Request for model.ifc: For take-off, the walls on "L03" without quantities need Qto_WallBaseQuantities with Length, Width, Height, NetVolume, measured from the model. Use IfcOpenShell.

First a look at what the model holds.

```python
import ifcopenshell
import ifcopenshell.util.element
import ifcopenshell.util.unit

model = ifcopenshell.open("model.ifc")
print(model.schema)
for unit_type in ("LENGTHUNIT", "AREAUNIT", "VOLUMEUNIT"):
    print(unit_type, ifcopenshell.util.unit.calculate_unit_scale(model, unit_type))
storey = next(s for s in model.by_type("IfcBuildingStorey") if s.Name == "L03")
walls = [e for e in ifcopenshell.util.element.get_decomposition(storey) if e.is_a("IfcWall")]
for e in sorted(walls, key=lambda e: e.id()):
    print(e.id(), e.is_a(), e.Name, list(ifcopenshell.util.element.get_psets(e, qtos_only=True)), sep=" | ")
```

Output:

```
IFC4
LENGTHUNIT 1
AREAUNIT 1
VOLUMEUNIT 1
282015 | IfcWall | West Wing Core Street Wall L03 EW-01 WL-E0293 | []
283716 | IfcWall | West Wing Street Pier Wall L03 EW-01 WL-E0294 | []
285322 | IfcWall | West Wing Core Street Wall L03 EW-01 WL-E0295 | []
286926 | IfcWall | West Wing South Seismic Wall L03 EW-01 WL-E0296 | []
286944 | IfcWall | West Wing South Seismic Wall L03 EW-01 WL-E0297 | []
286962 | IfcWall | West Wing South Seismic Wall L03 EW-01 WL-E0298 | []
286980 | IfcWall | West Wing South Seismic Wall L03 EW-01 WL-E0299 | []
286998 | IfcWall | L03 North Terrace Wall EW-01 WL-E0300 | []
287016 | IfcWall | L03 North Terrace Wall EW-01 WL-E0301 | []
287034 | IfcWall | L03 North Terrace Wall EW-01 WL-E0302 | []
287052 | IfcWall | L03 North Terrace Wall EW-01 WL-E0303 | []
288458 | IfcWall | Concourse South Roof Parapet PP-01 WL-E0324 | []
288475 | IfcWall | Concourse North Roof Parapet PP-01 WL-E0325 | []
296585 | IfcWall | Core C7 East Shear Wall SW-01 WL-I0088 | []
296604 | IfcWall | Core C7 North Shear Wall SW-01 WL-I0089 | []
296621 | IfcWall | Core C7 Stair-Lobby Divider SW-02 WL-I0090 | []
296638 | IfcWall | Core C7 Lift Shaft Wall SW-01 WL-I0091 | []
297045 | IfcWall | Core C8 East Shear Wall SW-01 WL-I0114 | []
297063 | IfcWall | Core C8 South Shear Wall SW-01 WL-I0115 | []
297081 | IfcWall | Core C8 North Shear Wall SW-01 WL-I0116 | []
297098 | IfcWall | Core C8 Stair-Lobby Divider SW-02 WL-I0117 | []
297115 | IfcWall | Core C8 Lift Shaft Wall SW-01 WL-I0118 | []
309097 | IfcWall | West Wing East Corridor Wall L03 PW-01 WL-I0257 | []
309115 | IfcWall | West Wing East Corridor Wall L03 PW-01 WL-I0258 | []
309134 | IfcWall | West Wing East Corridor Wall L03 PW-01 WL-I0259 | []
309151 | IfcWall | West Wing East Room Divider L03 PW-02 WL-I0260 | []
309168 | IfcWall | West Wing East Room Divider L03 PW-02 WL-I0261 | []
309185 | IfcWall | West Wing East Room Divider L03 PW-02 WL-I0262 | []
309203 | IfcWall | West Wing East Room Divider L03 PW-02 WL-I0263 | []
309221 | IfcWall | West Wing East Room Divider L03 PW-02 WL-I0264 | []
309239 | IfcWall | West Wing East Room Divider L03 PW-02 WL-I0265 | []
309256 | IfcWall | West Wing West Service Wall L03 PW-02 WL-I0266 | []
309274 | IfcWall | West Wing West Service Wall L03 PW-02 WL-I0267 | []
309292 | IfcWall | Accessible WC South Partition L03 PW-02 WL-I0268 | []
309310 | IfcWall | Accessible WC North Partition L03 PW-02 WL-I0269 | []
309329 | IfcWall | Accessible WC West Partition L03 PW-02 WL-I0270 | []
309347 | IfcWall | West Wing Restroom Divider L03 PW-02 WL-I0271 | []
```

```python
import ifcopenshell
import ifcopenshell.api.pset
import ifcopenshell.geom
import ifcopenshell.util.element
import ifcopenshell.util.shape
import ifcopenshell.util.unit

model = ifcopenshell.open("model.ifc")
unit_scale = ifcopenshell.util.unit.calculate_unit_scale(model)
volume_scale = ifcopenshell.util.unit.calculate_unit_scale(model, "VOLUMEUNIT")
settings = ifcopenshell.geom.settings()

storey = next(s for s in model.by_type("IfcBuildingStorey") if s.Name == "L03")
walls = [e for e in ifcopenshell.util.element.get_decomposition(storey) if e.is_a("IfcWall")]

for e in sorted(walls, key=lambda e: e.id()):
    if ifcopenshell.util.element.get_psets(e, qtos_only=True, should_inherit=False):
        continue
    # Geometry comes back in metres, in the element's own axes.
    shape = ifcopenshell.geom.create_shape(settings, e)
    values = {
        "Length": ifcopenshell.util.shape.get_x(shape.geometry) / unit_scale,
        "Width": ifcopenshell.util.shape.get_y(shape.geometry) / unit_scale,
        "Height": ifcopenshell.util.shape.get_z(shape.geometry) / unit_scale,
        "NetVolume": ifcopenshell.util.shape.get_volume(shape.geometry) / volume_scale,
    }
    qto = ifcopenshell.api.pset.add_qto(model, product=e, name="Qto_WallBaseQuantities")
    ifcopenshell.api.pset.edit_qto(model, qto=qto, properties=values)
    print(e.id(), {k: round(v, 3) for k, v in values.items()})

model.write("model-out.ifc")
```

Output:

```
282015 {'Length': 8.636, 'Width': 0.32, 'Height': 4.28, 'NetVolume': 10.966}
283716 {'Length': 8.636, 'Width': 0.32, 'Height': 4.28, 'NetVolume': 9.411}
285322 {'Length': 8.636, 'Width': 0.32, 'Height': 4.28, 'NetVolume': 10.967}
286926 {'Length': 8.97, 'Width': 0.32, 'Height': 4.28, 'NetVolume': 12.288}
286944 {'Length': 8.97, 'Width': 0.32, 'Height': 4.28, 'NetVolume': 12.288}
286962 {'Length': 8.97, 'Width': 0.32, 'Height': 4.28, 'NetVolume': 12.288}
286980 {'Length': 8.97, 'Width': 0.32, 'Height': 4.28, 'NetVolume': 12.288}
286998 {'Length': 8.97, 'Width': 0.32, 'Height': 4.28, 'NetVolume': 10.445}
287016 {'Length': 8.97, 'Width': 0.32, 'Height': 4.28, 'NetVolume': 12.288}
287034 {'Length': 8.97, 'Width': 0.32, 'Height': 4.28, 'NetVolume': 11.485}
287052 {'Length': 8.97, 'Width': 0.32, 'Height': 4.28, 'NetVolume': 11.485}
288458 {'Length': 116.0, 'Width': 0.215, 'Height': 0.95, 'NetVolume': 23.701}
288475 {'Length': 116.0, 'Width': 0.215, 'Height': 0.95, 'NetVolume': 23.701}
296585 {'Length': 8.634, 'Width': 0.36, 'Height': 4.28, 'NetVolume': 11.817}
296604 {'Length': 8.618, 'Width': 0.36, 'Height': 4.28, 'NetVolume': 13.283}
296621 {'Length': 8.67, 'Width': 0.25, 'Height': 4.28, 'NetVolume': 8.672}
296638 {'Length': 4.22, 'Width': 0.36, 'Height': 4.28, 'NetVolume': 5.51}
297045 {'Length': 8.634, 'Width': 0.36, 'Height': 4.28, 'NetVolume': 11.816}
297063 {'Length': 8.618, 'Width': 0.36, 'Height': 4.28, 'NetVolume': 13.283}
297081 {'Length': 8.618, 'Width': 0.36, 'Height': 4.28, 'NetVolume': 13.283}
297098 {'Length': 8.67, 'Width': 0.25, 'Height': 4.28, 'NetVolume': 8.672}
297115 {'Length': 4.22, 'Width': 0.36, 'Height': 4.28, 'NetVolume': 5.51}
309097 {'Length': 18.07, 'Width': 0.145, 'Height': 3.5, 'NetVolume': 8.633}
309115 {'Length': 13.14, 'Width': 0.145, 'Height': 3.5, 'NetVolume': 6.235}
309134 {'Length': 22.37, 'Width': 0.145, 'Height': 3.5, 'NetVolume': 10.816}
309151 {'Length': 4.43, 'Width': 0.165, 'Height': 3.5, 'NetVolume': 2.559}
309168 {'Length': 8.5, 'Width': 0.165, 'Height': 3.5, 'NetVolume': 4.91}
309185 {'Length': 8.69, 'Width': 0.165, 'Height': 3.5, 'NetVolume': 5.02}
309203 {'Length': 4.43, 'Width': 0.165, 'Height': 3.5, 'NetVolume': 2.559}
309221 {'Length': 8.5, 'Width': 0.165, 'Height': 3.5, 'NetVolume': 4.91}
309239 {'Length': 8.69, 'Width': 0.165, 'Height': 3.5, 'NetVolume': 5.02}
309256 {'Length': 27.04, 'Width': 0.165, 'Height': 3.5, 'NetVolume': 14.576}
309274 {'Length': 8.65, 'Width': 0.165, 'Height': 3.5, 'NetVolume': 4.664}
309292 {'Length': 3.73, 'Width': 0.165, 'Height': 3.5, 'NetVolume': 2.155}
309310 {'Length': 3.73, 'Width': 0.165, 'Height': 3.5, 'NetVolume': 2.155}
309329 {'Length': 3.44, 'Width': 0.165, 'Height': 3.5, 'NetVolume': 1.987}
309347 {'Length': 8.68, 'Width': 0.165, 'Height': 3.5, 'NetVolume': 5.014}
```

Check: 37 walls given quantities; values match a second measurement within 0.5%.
